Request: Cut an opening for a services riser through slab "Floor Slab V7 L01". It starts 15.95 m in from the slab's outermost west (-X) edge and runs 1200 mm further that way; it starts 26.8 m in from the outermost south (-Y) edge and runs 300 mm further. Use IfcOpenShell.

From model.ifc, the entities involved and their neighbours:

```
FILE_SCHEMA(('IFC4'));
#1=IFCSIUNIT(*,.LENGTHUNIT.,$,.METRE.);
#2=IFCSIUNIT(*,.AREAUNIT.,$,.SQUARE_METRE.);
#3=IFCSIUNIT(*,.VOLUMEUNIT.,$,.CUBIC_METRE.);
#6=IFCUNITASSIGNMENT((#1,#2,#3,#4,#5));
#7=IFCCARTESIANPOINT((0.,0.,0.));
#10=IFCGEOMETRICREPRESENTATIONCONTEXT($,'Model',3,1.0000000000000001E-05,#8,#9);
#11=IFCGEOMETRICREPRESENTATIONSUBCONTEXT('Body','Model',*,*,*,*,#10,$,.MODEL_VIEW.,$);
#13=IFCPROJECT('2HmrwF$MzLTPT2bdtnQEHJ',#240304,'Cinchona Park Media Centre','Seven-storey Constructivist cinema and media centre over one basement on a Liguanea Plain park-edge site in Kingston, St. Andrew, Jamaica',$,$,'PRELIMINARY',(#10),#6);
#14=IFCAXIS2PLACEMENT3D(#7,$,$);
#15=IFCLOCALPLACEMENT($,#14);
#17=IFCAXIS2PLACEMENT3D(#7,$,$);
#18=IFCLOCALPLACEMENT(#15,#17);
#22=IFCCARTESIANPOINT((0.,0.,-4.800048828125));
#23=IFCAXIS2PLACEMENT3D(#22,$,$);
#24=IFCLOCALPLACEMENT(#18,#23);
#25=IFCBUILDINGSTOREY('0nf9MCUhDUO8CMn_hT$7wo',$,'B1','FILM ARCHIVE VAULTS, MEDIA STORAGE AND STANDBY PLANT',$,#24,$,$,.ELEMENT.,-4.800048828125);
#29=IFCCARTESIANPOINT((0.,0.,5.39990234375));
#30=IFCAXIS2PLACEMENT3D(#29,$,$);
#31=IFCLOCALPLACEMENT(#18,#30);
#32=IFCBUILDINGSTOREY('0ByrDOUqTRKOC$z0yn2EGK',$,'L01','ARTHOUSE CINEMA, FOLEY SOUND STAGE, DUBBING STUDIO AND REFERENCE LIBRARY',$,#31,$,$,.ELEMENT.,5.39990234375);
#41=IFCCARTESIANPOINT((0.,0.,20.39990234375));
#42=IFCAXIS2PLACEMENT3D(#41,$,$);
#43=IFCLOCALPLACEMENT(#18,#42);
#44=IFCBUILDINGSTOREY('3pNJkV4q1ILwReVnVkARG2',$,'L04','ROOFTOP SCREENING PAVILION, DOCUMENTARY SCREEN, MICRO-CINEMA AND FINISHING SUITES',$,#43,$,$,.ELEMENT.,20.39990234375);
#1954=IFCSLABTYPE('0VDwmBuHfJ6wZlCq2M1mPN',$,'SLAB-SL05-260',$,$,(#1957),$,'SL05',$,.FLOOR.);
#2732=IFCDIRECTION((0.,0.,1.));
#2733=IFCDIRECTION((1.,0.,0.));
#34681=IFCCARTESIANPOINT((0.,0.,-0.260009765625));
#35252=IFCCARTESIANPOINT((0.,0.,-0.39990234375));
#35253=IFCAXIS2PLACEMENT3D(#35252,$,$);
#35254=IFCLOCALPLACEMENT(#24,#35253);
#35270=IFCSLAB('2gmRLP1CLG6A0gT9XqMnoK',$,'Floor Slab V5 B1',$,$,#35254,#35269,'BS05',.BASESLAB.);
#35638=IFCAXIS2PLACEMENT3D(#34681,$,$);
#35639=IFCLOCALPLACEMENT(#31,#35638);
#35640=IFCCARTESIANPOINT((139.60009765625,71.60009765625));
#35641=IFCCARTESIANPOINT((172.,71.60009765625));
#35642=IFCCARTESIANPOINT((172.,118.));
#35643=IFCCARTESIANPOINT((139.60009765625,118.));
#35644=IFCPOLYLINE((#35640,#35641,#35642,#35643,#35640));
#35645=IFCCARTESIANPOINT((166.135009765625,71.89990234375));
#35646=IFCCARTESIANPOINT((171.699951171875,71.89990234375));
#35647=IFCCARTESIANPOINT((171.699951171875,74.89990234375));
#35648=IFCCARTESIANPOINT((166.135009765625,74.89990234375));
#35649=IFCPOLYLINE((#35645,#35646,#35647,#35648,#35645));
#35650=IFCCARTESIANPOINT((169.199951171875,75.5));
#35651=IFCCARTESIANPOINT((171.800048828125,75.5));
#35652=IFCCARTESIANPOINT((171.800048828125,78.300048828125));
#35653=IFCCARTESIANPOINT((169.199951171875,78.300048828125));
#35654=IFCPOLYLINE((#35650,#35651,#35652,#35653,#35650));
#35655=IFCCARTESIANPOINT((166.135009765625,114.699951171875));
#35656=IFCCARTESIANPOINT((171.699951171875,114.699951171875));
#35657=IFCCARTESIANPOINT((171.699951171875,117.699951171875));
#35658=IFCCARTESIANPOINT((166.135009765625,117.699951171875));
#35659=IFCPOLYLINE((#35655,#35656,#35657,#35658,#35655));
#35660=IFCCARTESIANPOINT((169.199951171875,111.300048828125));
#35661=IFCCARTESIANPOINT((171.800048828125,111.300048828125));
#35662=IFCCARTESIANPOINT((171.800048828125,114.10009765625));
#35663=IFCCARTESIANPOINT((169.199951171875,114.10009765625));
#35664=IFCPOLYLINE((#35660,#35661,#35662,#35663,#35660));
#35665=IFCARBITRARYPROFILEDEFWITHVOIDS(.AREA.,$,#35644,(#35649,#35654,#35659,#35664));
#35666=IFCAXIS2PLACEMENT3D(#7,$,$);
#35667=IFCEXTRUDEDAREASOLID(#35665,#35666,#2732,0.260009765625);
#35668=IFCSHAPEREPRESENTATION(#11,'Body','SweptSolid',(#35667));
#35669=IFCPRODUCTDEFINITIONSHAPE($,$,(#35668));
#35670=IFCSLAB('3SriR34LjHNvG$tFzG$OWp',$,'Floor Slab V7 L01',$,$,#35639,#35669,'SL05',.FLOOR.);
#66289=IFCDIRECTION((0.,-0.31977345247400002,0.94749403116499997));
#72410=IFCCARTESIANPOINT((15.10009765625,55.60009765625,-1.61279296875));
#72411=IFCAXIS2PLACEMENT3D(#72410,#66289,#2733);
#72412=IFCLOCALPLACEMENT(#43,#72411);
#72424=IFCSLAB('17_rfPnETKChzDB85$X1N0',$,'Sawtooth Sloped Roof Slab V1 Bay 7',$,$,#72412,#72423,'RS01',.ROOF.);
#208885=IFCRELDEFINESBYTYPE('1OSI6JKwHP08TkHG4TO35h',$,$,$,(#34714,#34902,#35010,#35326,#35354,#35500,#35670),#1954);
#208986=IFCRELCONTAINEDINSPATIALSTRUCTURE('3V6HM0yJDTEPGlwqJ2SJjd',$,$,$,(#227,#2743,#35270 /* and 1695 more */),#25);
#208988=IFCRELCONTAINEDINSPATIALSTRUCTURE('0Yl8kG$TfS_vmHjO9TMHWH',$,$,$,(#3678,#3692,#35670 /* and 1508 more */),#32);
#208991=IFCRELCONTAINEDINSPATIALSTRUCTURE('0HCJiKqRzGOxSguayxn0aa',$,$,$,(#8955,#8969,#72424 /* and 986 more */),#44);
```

```python
import numpy as np
import ifcopenshell
import ifcopenshell.api.feature
import ifcopenshell.api.geometry
import ifcopenshell.api.root
import ifcopenshell.geom
import ifcopenshell.util.placement
import ifcopenshell.util.representation
import ifcopenshell.util.shape
import ifcopenshell.util.unit

model = ifcopenshell.open("model.ifc")
unit_scale = ifcopenshell.util.unit.calculate_unit_scale(model)
settings = ifcopenshell.geom.settings()


def volume(element):
    """Net volume in cubic metres, openings subtracted."""
    shape = ifcopenshell.geom.create_shape(settings, element)
    return ifcopenshell.util.shape.get_volume(shape.geometry)


slab = model.by_guid("3SriR34LjHNvG$tFzG$OWp")
before = volume(slab)

# Extent in the slab's own axes, in metres. The edges named are its -X and -Y sides.
slab_shape = ifcopenshell.geom.create_shape(settings, slab)
vertices = ifcopenshell.util.shape.get_vertices(slab_shape.geometry)
x_min, y_min, bottom = vertices.min(axis=0)
top = vertices[:, 2].max()

opening = ifcopenshell.api.root.create_entity(model, ifc_class="IfcOpeningElement", name="Services riser opening", predefined_type="OPENING")
context = ifcopenshell.util.representation.get_context(model, "Model", "Body", "MODEL_VIEW")
width, depth = 1.2, 0.3
outline = [(0.0, 0.0), (width, 0.0), (width, depth), (0.0, depth), (0.0, 0.0)]
# Overshoot both faces by 50 mm so the cut is clean.
shape = ifcopenshell.api.geometry.add_slab_representation(
    model, context=context, depth=top - bottom + 0.1, polyline=outline
)
ifcopenshell.api.geometry.assign_representation(model, product=opening, representation=shape)

matrix = ifcopenshell.util.placement.get_local_placement(slab.ObjectPlacement)
matrix[:, 3] = matrix @ np.append(np.array([x_min + 15.95, y_min + 26.8, bottom - 0.05]) / unit_scale, 1.0)
ifcopenshell.api.geometry.edit_object_placement(model, product=opening, matrix=matrix, is_si=False)
ifcopenshell.api.feature.add_feature(model, feature=opening, element=slab)

after = volume(slab)

print(f"slab volume {before:.3f} -> {after:.3f} m3")

model.write("model_edited.ifc")
```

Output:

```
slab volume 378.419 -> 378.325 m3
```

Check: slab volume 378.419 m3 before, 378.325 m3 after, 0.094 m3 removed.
